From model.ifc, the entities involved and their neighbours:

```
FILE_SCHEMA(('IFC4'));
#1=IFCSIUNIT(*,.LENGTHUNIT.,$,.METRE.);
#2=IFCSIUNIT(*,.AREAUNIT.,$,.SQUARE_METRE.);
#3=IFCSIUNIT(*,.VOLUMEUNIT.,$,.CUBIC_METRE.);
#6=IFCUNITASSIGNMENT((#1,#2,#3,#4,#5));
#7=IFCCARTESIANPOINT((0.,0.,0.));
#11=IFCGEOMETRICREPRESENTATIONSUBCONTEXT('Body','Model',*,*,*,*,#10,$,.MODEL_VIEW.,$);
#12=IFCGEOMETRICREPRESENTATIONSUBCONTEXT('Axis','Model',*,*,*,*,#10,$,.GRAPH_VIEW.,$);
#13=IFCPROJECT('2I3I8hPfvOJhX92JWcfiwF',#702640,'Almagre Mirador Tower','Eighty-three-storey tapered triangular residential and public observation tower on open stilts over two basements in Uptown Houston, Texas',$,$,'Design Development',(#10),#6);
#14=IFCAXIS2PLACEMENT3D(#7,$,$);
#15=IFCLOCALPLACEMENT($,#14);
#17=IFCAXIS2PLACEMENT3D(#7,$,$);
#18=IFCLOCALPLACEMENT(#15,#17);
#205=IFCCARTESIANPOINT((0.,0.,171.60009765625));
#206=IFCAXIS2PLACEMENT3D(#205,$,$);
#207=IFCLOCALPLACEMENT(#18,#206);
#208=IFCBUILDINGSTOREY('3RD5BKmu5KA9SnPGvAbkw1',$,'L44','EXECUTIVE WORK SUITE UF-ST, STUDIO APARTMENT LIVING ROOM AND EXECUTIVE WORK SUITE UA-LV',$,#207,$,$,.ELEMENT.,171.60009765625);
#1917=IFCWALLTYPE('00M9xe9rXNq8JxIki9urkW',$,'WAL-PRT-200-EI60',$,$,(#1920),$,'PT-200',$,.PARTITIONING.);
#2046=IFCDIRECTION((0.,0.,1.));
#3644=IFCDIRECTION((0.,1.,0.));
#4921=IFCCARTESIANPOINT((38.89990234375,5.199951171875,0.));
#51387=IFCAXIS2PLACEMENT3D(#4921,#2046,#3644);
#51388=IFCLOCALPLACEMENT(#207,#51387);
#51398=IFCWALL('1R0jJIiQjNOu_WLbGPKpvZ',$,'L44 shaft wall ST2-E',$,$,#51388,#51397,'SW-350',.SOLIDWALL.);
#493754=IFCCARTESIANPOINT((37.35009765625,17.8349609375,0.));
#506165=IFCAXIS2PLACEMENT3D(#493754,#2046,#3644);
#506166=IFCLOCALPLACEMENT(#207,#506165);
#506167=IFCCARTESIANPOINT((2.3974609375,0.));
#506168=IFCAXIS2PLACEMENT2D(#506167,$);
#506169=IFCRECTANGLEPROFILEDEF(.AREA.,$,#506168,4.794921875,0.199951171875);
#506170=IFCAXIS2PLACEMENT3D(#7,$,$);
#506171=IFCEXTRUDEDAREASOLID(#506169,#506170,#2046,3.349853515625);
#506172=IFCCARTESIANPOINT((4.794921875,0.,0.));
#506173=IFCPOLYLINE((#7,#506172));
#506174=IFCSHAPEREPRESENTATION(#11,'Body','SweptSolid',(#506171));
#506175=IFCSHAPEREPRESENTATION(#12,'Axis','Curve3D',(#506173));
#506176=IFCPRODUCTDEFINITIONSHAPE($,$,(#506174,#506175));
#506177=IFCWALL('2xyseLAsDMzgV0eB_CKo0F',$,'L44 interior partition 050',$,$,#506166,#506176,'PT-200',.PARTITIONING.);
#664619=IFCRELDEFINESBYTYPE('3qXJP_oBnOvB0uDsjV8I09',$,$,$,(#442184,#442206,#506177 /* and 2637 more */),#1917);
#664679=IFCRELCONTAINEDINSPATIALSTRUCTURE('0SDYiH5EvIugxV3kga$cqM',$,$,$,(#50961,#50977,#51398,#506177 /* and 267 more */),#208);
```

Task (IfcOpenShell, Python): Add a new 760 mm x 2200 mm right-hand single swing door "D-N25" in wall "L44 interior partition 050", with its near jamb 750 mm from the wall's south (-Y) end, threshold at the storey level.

```python
import numpy as np
import ifcopenshell
import ifcopenshell.api.feature
import ifcopenshell.api.geometry
import ifcopenshell.api.root
import ifcopenshell.api.spatial
import ifcopenshell.geom
import ifcopenshell.util.element
import ifcopenshell.util.placement
import ifcopenshell.util.representation
import ifcopenshell.util.shape
import ifcopenshell.util.unit

model = ifcopenshell.open("model.ifc")
unit_scale = ifcopenshell.util.unit.calculate_unit_scale(model)
settings = ifcopenshell.geom.settings()


def volume(element):
    """Net volume in cubic metres, openings subtracted."""
    shape = ifcopenshell.geom.create_shape(settings, element)
    return ifcopenshell.util.shape.get_volume(shape.geometry)


wall = model.by_guid("2xyseLAsDMzgV0eB_CKo0F")
storey = ifcopenshell.util.element.get_container(wall, ifc_class="IfcBuildingStorey")
context = ifcopenshell.util.representation.get_context(model, "Model", "Body", "MODEL_VIEW")
before = volume(wall)

width, height, from_end, sill = 0.76, 2.2, 0.75, 0.0  # metres

# The wall runs along its own X axis, and the end named is its -X end.
wall_shape = ifcopenshell.geom.create_shape(settings, wall)
x, y, z = ifcopenshell.util.shape.get_vertices(wall_shape.geometry).T
start = x.min() + from_end
face, thickness = float(y.min()), float(y.max() - y.min())
wall_matrix = ifcopenshell.util.placement.get_local_placement(wall.ObjectPlacement)
level = ifcopenshell.util.placement.get_local_placement(storey.ObjectPlacement)[2, 3]


def in_wall(x, y):
    """Placement at x, y metres in the wall's axes, at sill height."""
    matrix = wall_matrix.copy()
    matrix[:, 3] = wall_matrix @ np.array([x / unit_scale, y / unit_scale, 0.0, 1.0])
    matrix[2, 3] = level + sill / unit_scale
    return matrix


# Opening: a box that overshoots both wall faces by 50 mm.
opening = ifcopenshell.api.root.create_entity(model, ifc_class="IfcOpeningElement", predefined_type="OPENING")
box = ifcopenshell.api.geometry.add_wall_representation(
    model, context=context, length=width, height=height, thickness=thickness + 0.1
)
ifcopenshell.api.geometry.assign_representation(model, product=opening, representation=box)
ifcopenshell.api.geometry.edit_object_placement(model, product=opening, matrix=in_wall(start, face - 0.05), is_si=False)
ifcopenshell.api.feature.add_feature(model, feature=opening, element=wall)

door = ifcopenshell.api.root.create_entity(model, ifc_class="IfcDoor", name="D-N25", predefined_type="DOOR")
door.OverallWidth, door.OverallHeight = width / unit_scale, height / unit_scale
door.OperationType = "SINGLE_SWING_RIGHT"
body = ifcopenshell.api.geometry.add_door_representation(
    model,
    context=context,
    overall_width=door.OverallWidth,
    overall_height=door.OverallHeight,
    operation_type="SINGLE_SWING_RIGHT",
    lining_properties={"LiningDepth": thickness / unit_scale, "ThresholdDepth": thickness / unit_scale},
)
ifcopenshell.api.geometry.assign_representation(model, product=door, representation=body)
ifcopenshell.api.spatial.assign_container(model, products=[door], relating_structure=storey)
ifcopenshell.api.feature.add_filling(model, opening=opening, element=door)

# The lining spans the wall, so the door starts at the wall face.
ifcopenshell.api.geometry.edit_object_placement(model, product=door, matrix=in_wall(start, face), is_si=False)

after = volume(wall)

print(f"wall volume {before:.3f} -> {after:.3f} m3")

model.write("model_updated.ifc")
```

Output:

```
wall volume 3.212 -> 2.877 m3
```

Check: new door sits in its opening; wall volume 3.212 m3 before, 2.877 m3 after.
